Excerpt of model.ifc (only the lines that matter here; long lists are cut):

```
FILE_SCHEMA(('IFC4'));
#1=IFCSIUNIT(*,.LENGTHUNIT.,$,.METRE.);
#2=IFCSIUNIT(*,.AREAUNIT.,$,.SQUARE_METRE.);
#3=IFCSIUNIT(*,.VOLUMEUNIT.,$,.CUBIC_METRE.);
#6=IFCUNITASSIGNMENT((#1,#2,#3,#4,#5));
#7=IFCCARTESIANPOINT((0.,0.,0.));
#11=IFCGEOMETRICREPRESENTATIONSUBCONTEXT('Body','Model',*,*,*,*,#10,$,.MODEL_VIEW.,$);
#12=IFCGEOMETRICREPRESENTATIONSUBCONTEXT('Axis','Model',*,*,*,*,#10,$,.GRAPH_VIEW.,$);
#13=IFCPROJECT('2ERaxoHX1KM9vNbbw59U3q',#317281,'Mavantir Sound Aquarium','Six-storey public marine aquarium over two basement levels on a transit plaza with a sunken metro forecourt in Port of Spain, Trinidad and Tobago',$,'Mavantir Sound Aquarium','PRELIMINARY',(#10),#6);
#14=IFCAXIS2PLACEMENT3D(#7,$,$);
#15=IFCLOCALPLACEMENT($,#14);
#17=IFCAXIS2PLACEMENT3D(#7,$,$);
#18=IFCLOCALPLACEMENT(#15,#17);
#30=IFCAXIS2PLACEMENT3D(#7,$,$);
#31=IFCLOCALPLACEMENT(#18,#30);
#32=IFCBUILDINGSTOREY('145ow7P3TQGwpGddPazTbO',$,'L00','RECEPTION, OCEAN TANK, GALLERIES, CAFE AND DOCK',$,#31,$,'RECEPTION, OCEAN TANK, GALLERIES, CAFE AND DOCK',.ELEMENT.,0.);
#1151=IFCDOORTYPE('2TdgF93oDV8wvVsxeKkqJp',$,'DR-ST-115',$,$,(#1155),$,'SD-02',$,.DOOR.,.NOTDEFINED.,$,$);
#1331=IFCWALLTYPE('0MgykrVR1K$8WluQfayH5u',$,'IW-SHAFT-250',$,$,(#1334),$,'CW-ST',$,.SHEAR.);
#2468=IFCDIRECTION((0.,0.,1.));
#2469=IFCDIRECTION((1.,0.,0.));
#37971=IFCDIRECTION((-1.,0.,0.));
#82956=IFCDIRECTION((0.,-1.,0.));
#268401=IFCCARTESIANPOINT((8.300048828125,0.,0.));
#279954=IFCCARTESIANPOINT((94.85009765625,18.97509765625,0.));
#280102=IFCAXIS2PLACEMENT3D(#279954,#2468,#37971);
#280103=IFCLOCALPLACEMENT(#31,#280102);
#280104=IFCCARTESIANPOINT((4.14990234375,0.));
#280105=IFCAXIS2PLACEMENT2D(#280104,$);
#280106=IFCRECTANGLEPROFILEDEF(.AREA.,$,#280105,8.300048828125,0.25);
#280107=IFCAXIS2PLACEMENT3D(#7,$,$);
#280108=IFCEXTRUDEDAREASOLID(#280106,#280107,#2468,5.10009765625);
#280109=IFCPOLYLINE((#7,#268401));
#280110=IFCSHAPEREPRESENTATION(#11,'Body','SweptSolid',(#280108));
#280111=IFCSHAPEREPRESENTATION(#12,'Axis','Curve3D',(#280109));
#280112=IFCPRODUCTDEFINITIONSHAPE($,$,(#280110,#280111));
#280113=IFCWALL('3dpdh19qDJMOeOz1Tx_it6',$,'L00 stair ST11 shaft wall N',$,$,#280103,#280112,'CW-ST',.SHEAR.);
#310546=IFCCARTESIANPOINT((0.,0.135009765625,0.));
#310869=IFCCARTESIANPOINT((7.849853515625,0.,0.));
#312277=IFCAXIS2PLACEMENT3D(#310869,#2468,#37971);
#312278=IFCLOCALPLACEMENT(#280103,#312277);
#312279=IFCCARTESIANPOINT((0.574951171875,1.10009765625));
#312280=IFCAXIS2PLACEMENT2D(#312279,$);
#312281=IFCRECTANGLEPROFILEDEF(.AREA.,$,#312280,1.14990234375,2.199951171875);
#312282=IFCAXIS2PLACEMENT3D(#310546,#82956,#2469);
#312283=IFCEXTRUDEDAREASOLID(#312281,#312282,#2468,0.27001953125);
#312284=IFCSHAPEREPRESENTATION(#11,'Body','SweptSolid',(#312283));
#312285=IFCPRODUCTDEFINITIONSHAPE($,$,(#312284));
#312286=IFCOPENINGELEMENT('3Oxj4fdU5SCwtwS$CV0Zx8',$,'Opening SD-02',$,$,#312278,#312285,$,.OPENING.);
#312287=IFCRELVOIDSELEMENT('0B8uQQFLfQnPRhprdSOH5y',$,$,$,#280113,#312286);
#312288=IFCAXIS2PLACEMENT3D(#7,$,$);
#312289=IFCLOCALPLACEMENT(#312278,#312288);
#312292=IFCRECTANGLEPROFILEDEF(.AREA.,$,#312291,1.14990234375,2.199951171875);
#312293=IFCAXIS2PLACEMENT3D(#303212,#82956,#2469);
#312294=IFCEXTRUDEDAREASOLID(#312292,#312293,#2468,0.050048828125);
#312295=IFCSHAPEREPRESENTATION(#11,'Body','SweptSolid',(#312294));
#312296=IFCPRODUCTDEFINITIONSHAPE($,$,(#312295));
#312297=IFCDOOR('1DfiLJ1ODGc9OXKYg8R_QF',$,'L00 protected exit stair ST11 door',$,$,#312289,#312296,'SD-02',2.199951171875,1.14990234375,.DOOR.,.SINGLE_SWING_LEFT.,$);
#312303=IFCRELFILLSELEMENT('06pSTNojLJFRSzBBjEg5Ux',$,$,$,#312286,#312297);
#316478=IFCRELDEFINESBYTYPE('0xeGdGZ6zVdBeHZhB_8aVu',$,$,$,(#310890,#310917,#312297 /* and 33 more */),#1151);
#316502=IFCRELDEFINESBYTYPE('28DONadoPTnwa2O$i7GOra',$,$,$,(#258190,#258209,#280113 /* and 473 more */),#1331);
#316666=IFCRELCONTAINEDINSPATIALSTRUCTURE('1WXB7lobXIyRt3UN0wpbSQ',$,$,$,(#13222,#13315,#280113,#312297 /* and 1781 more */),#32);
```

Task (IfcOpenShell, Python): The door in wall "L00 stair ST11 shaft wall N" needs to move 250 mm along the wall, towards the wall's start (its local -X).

```python
import ifcopenshell
import ifcopenshell.api.geometry
import ifcopenshell.util.placement
import ifcopenshell.util.unit

model = ifcopenshell.open("model.ifc")
unit_scale = ifcopenshell.util.unit.calculate_unit_scale(model)

door = model.by_guid("1DfiLJ1ODGc9OXKYg8R_QF")
opening = door.FillsVoids[0].RelatingOpeningElement
wall = opening.VoidsElements[0].RelatingBuildingElement

wall_matrix = ifcopenshell.util.placement.get_local_placement(wall.ObjectPlacement)
shift = wall_matrix[:3, 0] * -0.25 / unit_scale
before = ifcopenshell.util.placement.get_local_placement(door.ObjectPlacement)[:3, 3].copy()

# The door is placed relative to its opening, so it follows when the opening moves.
matrix = ifcopenshell.util.placement.get_local_placement(opening.ObjectPlacement)
matrix[:3, 3] += shift
ifcopenshell.api.geometry.edit_object_placement(
    model, product=opening, matrix=matrix, is_si=False, should_transform_children=True
)

after = ifcopenshell.util.placement.get_local_placement(door.ObjectPlacement)[:3, 3]
print("door moved by", (after - before).round(3) + 0.0)

model.write("model_updated.ifc")
```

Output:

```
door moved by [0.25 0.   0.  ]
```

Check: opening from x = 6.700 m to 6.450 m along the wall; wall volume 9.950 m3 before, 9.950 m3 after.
